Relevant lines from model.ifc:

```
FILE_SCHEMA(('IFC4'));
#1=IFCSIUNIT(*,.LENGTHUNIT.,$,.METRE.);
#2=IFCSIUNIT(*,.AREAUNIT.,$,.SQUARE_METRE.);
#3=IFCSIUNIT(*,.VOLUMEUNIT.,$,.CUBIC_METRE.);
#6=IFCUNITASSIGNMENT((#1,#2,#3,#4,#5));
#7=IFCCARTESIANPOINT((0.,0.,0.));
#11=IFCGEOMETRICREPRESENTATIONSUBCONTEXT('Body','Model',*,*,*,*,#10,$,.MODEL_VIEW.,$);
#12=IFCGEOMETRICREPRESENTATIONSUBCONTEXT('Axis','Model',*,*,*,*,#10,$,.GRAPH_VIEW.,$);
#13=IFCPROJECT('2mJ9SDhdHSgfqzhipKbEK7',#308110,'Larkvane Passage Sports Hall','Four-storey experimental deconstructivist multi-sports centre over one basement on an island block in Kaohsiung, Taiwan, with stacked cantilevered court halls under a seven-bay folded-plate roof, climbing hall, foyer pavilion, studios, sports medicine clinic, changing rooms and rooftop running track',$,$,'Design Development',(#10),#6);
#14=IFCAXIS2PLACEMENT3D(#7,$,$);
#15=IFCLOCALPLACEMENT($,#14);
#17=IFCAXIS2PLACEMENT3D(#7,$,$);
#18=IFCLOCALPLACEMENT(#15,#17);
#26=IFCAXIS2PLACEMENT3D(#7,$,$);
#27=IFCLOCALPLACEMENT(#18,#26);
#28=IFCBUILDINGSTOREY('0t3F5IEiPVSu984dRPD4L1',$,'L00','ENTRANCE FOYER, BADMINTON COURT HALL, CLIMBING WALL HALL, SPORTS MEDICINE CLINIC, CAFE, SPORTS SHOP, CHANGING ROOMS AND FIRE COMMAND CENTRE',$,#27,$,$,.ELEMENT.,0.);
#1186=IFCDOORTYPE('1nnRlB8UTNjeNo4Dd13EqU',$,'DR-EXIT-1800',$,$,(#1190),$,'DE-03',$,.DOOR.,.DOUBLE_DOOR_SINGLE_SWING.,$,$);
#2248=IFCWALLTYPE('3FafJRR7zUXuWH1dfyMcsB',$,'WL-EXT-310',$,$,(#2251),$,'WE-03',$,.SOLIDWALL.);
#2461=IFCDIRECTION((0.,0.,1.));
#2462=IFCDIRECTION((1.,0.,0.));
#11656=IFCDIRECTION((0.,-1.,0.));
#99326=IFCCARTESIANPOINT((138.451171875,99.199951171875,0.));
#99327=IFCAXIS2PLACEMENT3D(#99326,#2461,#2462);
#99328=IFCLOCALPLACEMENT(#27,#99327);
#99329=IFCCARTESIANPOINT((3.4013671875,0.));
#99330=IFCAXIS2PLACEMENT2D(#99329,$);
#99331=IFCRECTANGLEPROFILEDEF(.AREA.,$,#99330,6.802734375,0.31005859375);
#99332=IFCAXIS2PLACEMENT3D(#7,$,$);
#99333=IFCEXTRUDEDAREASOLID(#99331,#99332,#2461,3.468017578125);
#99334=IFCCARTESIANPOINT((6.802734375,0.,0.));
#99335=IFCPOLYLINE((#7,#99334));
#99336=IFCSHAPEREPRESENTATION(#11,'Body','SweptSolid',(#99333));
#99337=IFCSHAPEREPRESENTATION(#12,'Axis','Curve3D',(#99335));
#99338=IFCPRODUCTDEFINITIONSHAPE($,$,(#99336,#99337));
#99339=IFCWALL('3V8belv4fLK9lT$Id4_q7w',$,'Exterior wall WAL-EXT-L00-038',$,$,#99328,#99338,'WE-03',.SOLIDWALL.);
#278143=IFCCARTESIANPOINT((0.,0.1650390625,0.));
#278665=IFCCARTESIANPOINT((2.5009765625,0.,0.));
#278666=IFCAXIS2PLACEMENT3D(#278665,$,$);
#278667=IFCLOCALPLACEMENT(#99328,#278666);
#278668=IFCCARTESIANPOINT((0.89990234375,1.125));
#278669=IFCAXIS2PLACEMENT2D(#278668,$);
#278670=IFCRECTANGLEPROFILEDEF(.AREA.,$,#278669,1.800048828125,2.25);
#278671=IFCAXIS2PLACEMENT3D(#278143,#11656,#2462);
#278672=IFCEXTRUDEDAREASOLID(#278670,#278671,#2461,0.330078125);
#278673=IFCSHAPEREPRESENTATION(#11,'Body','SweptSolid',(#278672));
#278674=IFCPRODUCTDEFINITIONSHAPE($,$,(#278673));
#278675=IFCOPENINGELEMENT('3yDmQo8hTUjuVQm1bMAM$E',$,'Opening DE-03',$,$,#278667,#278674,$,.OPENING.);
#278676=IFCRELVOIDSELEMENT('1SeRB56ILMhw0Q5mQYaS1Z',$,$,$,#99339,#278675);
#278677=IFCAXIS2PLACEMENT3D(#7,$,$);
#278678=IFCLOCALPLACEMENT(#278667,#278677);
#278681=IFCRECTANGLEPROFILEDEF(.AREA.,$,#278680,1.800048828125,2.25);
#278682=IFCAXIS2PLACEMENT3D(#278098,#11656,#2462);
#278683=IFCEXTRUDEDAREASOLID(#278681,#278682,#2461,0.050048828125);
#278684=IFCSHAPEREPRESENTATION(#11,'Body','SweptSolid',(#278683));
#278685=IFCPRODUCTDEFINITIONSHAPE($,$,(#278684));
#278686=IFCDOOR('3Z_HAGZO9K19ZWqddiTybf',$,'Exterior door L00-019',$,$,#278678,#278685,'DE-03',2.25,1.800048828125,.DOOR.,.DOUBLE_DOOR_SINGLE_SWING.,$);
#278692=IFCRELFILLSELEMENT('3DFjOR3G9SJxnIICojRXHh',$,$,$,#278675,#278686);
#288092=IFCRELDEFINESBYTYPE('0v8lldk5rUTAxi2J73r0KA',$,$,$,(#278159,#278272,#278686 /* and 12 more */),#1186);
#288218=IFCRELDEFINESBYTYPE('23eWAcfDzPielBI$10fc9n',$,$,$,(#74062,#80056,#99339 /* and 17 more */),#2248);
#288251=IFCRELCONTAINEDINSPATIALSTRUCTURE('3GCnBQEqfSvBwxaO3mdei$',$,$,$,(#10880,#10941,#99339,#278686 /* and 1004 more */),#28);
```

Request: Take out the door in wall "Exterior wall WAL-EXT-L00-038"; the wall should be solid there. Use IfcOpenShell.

```python
import ifcopenshell
import ifcopenshell.api.feature
import ifcopenshell.api.root
import ifcopenshell.geom
import ifcopenshell.util.shape

model = ifcopenshell.open("model.ifc")
settings = ifcopenshell.geom.settings()


def volume(element):
    """Net volume in cubic metres, openings subtracted."""
    shape = ifcopenshell.geom.create_shape(settings, element)
    return ifcopenshell.util.shape.get_volume(shape.geometry)


door = model.by_id(278686)
opening = door.FillsVoids[0].RelatingOpeningElement
wall = opening.VoidsElements[0].RelatingBuildingElement
before = volume(wall)

ifcopenshell.api.root.remove_product(model, product=door)
ifcopenshell.api.feature.remove_feature(model, feature=opening)

after = volume(wall)

print(f"wall volume {before:.3f} -> {after:.3f} m3")

model.write("model_edited.ifc")
```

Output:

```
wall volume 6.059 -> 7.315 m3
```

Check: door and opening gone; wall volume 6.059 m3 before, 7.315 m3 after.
